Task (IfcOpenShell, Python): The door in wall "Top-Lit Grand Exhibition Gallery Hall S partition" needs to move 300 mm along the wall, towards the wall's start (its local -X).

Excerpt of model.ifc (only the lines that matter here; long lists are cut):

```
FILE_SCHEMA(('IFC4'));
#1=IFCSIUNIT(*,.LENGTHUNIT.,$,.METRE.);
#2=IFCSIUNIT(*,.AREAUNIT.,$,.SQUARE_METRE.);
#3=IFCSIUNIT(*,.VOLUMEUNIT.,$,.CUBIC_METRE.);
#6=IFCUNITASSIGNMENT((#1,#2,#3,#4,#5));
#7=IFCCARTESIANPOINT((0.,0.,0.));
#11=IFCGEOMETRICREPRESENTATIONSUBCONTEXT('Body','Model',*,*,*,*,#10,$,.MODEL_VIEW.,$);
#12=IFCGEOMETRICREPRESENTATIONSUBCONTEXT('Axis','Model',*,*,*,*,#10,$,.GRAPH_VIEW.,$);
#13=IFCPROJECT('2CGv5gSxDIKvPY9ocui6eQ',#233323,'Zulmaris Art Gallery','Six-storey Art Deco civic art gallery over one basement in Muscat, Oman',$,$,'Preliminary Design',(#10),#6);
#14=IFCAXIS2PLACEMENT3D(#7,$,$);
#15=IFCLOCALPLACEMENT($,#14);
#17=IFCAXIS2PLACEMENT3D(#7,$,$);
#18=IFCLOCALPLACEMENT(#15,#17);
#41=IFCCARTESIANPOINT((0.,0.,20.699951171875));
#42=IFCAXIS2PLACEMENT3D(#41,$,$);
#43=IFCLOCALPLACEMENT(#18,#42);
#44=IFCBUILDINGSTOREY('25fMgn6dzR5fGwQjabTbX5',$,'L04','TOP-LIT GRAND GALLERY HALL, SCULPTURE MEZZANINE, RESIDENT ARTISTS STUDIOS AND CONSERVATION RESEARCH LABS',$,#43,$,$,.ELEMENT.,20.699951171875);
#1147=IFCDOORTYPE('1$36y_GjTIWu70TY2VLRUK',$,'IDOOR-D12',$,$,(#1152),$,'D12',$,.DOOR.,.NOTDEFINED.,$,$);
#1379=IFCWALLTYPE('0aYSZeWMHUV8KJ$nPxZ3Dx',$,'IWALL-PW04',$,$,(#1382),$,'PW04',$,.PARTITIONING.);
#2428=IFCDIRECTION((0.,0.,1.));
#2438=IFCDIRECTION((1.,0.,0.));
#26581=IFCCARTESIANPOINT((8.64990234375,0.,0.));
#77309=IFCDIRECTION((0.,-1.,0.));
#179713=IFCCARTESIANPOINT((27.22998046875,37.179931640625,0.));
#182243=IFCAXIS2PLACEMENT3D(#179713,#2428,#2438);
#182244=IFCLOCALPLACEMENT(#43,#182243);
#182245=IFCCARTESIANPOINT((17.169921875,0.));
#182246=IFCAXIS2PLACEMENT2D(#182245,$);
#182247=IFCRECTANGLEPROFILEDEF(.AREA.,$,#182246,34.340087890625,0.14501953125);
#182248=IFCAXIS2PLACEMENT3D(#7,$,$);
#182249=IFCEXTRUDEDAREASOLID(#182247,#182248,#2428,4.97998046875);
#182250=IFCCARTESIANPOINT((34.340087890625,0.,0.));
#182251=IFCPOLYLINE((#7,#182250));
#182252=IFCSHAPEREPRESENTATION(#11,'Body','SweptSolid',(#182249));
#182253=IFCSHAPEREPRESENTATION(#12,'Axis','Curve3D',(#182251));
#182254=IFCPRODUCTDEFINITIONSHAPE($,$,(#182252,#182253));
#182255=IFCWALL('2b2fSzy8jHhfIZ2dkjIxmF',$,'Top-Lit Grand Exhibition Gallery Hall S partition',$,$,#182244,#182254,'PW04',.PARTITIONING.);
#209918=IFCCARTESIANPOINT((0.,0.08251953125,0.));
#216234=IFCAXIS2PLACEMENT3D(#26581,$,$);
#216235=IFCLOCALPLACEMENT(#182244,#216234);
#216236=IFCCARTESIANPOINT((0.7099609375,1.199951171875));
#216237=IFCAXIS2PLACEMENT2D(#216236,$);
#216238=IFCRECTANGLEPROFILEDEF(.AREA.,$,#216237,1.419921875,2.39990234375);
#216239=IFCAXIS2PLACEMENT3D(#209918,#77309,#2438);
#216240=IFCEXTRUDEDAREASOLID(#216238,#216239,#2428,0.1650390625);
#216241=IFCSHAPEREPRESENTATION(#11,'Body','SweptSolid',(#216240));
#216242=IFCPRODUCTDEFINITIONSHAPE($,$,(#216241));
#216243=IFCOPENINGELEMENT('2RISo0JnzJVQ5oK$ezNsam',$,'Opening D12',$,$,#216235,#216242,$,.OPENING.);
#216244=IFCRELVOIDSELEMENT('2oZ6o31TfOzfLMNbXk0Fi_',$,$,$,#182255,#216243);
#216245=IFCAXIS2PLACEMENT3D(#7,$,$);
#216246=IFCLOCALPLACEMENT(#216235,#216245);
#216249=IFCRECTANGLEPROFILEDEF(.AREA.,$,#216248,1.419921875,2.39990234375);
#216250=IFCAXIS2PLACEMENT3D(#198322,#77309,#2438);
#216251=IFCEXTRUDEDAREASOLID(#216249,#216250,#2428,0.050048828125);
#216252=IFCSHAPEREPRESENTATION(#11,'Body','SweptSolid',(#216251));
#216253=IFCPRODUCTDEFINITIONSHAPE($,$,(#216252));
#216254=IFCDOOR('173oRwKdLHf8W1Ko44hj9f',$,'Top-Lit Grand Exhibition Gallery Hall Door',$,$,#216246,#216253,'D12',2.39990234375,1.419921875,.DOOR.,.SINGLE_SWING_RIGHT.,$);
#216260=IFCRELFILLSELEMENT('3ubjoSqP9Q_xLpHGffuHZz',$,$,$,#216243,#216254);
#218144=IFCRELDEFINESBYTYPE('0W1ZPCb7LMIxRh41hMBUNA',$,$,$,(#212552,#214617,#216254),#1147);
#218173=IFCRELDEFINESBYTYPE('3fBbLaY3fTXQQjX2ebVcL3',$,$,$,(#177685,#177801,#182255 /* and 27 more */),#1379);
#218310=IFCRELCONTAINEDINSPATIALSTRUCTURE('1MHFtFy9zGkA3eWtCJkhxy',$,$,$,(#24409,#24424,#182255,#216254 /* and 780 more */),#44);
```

```python
import ifcopenshell
import ifcopenshell.api.geometry
import ifcopenshell.util.placement

model = ifcopenshell.open("model.ifc")

door = model.by_guid("173oRwKdLHf8W1Ko44hj9f")
opening = door.FillsVoids[0].RelatingOpeningElement
wall = opening.VoidsElements[0].RelatingBuildingElement

wall_matrix = ifcopenshell.util.placement.get_local_placement(wall.ObjectPlacement)
shift = wall_matrix[:3, 0] * -0.3
before = ifcopenshell.util.placement.get_local_placement(door.ObjectPlacement)[:3, 3].copy()

# The door is placed relative to its opening, so it follows when the opening moves.
matrix = ifcopenshell.util.placement.get_local_placement(opening.ObjectPlacement)
matrix[:3, 3] += shift
ifcopenshell.api.geometry.edit_object_placement(
    model, product=opening, matrix=matrix, is_si=False, should_transform_children=True
)

after = ifcopenshell.util.placement.get_local_placement(door.ObjectPlacement)[:3, 3]
print("door moved by", (after - before).round(3) + 0.0)

model.write("model-out.ifc")
```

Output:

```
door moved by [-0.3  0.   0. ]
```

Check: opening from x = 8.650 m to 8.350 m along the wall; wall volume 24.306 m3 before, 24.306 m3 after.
